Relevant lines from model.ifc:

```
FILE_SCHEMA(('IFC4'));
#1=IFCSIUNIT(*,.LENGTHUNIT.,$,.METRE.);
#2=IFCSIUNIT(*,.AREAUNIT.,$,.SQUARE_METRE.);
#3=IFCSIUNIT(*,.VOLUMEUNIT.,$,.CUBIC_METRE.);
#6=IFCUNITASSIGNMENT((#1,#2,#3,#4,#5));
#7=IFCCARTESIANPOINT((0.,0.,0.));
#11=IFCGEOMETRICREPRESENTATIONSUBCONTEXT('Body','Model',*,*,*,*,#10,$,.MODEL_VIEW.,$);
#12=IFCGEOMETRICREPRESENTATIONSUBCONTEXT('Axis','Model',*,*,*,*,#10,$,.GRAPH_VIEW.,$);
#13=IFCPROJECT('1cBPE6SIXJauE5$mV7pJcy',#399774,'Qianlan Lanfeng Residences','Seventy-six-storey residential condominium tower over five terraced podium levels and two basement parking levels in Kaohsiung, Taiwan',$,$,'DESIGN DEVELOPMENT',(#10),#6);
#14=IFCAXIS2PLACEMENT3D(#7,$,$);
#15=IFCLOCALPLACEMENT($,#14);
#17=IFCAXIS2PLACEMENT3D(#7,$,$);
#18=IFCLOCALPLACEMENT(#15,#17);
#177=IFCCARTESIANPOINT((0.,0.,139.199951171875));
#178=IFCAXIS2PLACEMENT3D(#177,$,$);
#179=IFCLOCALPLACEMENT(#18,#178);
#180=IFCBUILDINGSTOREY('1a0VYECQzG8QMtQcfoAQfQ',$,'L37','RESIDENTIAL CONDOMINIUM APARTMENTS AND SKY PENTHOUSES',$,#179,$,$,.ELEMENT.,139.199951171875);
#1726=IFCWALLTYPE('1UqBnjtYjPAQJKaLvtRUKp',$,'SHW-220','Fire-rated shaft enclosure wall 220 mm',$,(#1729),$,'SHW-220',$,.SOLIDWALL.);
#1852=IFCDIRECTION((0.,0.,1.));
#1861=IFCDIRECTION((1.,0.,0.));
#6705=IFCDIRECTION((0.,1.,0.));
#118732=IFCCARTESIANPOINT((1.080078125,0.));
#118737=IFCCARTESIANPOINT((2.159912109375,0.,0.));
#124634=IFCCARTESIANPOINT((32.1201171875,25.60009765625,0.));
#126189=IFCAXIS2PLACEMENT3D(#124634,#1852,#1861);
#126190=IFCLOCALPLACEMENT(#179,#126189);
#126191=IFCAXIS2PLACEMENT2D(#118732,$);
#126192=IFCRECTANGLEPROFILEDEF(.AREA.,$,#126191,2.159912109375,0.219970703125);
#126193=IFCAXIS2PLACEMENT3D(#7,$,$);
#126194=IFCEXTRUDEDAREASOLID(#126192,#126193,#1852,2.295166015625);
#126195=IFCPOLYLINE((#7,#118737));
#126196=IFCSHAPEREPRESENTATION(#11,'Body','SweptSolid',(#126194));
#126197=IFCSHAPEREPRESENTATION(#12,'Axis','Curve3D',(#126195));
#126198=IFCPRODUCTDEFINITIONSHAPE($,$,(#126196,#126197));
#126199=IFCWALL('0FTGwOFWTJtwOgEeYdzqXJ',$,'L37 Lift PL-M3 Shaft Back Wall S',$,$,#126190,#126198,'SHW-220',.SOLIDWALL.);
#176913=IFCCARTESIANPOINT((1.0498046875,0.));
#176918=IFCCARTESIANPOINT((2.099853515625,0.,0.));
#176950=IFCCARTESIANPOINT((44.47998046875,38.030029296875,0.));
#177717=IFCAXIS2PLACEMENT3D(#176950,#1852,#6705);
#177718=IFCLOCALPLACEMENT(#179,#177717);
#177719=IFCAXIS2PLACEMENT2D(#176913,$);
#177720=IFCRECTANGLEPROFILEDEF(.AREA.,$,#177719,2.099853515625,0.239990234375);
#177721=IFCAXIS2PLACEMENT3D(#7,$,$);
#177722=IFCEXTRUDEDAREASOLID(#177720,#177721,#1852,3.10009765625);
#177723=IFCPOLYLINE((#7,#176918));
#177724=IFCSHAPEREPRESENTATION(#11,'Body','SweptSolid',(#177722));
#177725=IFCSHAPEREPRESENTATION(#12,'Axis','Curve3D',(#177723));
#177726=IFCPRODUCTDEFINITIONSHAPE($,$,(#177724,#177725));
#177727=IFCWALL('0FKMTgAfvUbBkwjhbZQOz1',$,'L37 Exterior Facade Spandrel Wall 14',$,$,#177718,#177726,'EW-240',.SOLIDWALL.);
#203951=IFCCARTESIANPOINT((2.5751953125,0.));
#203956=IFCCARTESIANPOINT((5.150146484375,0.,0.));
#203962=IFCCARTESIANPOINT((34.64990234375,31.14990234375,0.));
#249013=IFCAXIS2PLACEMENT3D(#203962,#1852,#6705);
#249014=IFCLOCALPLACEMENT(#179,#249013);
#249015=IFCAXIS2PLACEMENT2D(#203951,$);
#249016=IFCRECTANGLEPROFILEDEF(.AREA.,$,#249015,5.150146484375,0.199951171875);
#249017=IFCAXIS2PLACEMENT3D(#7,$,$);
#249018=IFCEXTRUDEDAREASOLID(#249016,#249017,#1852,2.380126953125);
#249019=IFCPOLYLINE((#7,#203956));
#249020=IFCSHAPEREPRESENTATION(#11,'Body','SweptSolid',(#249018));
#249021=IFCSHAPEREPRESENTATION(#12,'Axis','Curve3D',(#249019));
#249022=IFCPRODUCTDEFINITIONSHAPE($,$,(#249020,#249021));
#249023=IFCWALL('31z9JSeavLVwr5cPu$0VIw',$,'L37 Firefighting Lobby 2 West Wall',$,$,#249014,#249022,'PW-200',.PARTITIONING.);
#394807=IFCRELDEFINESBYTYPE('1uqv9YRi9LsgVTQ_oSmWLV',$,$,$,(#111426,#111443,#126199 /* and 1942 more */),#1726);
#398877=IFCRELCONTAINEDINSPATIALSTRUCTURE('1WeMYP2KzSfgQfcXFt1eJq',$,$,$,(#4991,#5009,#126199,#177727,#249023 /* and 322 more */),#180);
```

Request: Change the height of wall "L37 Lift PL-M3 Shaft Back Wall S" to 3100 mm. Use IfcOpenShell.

```python
import ifcopenshell
import ifcopenshell.geom
import ifcopenshell.util.representation
import ifcopenshell.util.shape
import ifcopenshell.util.unit

model = ifcopenshell.open("model.ifc")
unit_scale = ifcopenshell.util.unit.calculate_unit_scale(model)
settings = ifcopenshell.geom.settings()


def volume(element):
    """Net volume in cubic metres, openings subtracted."""
    shape = ifcopenshell.geom.create_shape(settings, element)
    return ifcopenshell.util.shape.get_volume(shape.geometry)


wall = model.by_id(126199)
before = volume(wall)

body = ifcopenshell.util.representation.get_representation(wall, "Model", "Body")
solid = body.Items[0]
old_height = solid.Depth
solid.Depth = 3.1 / unit_scale
after = volume(wall)

print(f"height {old_height:g} -> {solid.Depth:g}, volume {before:.3f} -> {after:.3f} m3")

model.write("model_edited.ifc")
```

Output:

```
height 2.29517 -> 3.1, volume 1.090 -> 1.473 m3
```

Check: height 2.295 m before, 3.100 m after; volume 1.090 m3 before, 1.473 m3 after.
